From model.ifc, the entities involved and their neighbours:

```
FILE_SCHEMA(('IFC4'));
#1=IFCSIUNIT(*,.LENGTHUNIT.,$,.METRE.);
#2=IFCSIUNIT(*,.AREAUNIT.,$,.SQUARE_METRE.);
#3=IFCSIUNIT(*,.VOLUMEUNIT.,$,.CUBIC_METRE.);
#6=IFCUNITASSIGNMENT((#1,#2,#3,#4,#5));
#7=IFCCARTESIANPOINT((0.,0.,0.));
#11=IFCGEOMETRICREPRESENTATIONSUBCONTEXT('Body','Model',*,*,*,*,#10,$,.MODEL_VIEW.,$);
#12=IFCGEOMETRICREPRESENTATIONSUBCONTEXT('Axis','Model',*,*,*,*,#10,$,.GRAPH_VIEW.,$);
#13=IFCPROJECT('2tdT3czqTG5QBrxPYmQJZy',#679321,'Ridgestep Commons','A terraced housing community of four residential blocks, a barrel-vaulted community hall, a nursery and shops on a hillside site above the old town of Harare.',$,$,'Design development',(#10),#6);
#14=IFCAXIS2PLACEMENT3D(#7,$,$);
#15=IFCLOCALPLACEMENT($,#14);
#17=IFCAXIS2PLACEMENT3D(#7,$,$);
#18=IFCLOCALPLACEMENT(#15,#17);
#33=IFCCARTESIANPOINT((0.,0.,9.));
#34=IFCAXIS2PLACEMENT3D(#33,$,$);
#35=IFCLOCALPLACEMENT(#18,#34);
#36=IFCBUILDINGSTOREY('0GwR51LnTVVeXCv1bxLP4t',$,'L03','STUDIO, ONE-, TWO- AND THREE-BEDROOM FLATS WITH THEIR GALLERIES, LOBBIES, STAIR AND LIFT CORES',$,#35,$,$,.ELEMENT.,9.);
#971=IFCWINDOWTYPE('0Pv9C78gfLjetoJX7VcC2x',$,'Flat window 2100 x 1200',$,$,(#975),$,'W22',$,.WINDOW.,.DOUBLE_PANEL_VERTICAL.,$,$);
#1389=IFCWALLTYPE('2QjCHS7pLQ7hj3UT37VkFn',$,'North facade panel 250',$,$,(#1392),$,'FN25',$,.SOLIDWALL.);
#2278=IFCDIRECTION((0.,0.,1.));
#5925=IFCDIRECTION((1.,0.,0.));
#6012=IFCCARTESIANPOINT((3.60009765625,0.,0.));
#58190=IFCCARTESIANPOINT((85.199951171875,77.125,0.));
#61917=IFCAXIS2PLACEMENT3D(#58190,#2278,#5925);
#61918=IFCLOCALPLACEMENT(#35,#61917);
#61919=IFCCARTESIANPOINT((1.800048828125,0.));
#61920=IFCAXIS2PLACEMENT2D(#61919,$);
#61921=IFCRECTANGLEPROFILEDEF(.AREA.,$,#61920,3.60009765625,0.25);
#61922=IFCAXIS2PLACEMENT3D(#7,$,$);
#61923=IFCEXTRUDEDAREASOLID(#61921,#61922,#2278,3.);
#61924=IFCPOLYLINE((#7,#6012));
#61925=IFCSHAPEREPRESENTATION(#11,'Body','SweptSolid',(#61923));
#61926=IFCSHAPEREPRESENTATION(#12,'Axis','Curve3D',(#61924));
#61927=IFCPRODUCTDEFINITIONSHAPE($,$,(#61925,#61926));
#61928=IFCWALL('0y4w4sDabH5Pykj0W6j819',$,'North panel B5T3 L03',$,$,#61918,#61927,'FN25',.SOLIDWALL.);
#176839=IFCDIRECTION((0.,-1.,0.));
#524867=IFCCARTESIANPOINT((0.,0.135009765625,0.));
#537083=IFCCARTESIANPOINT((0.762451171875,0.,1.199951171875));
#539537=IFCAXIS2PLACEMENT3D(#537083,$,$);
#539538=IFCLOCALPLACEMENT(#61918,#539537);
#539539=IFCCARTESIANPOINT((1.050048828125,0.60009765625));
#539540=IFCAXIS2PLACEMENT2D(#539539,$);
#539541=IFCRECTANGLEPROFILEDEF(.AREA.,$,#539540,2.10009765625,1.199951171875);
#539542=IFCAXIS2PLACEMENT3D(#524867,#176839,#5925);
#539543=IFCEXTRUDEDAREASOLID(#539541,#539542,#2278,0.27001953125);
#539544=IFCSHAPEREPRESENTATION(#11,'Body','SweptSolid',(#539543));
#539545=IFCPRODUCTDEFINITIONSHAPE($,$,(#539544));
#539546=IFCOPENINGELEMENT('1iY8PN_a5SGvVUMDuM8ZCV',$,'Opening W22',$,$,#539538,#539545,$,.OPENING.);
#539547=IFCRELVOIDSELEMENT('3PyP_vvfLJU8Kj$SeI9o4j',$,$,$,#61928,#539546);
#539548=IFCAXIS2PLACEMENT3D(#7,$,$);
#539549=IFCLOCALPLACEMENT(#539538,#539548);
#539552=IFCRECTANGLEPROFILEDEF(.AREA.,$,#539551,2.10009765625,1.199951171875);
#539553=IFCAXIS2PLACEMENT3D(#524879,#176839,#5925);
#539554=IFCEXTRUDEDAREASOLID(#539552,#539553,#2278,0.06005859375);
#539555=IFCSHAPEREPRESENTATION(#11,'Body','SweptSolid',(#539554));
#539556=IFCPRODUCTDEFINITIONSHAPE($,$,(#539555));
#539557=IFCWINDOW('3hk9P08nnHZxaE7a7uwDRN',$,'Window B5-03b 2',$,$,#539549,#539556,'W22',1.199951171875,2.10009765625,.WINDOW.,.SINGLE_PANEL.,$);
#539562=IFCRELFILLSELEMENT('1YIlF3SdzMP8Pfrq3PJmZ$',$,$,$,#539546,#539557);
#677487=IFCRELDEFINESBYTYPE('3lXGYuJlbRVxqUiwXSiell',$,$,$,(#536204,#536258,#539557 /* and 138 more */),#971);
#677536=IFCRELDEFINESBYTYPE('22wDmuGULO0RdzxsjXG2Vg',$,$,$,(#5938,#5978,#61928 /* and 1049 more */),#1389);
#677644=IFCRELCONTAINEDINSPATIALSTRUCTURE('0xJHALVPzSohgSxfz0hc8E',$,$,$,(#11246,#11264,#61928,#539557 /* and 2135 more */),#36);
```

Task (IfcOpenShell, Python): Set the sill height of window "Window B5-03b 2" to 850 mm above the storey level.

```python
import numpy as np
import ifcopenshell
import ifcopenshell.api.geometry
import ifcopenshell.geom
import ifcopenshell.util.element
import ifcopenshell.util.placement
import ifcopenshell.util.shape
import ifcopenshell.util.unit

model = ifcopenshell.open("model.ifc")
unit_scale = ifcopenshell.util.unit.calculate_unit_scale(model)

window = model.by_id(539557)
opening = window.FillsVoids[0].RelatingOpeningElement
storey = ifcopenshell.util.element.get_container(window, ifc_class="IfcBuildingStorey")
level = ifcopenshell.util.placement.get_local_placement(storey.ObjectPlacement)[2, 3]

# The opening's origin need not be at the sill, so measure its lowest point.
shape = ifcopenshell.geom.create_shape(ifcopenshell.geom.settings(), opening)
bottom = ifcopenshell.util.shape.get_shape_bottom_elevation(shape, shape.geometry) / unit_scale
dz = level + 0.85 - bottom

shift = np.array([0.0, 0.0, dz])
# The window is placed relative to its opening, so it follows when the opening moves.
matrix = ifcopenshell.util.placement.get_local_placement(opening.ObjectPlacement)
matrix[:3, 3] += shift
ifcopenshell.api.geometry.edit_object_placement(
    model, product=opening, matrix=matrix, is_si=False, should_transform_children=True
)

print(f"moved by {dz * unit_scale:+.3f} m")

model.write("model-out.ifc")
```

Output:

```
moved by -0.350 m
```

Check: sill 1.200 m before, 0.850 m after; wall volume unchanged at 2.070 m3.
